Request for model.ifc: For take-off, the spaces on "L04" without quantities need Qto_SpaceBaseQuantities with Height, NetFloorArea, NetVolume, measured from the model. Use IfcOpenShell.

First a look at what the model holds.

```python
import ifcopenshell
import ifcopenshell.util.element
import ifcopenshell.util.unit

model = ifcopenshell.open("model.ifc")
print(model.schema)
for unit_type in ("LENGTHUNIT", "AREAUNIT", "VOLUMEUNIT"):
    print(unit_type, ifcopenshell.util.unit.calculate_unit_scale(model, unit_type))
storey = next(s for s in model.by_type("IfcBuildingStorey") if s.Name == "L04")
spaces = [e for e in ifcopenshell.util.element.get_decomposition(storey) if e.is_a("IfcSpace")]
for e in sorted(spaces, key=lambda e: e.id()):
    print(e.id(), e.is_a(), e.Name, list(ifcopenshell.util.element.get_psets(e, qtos_only=True)), sep=" | ")
```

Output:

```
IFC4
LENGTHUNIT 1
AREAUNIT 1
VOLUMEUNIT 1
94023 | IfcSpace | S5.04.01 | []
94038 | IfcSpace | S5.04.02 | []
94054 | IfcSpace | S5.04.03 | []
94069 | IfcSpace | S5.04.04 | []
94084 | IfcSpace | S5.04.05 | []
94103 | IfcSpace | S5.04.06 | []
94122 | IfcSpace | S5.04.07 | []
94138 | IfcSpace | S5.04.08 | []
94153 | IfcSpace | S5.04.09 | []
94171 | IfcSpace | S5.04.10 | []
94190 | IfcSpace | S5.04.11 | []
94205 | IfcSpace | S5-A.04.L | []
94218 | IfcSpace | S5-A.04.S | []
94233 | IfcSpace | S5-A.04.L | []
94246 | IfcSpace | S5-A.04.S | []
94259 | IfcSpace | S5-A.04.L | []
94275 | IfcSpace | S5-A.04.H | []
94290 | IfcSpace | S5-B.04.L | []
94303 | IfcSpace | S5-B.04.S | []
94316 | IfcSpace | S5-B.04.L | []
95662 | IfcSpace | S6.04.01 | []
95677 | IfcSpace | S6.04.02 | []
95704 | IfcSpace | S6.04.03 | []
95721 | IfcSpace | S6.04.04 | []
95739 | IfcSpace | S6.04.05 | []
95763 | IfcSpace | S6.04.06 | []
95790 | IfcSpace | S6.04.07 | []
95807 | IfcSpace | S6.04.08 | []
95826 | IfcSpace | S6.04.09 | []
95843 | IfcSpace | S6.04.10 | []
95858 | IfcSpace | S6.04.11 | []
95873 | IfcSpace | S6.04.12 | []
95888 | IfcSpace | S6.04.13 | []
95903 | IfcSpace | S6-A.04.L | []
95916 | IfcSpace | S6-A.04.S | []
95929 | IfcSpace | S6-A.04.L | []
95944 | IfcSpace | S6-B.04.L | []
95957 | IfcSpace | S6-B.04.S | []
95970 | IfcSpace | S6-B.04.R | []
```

```python
import ifcopenshell
import ifcopenshell.api.pset
import ifcopenshell.geom
import ifcopenshell.util.element
import ifcopenshell.util.shape
import ifcopenshell.util.unit

model = ifcopenshell.open("model.ifc")
unit_scale = ifcopenshell.util.unit.calculate_unit_scale(model)
area_scale = ifcopenshell.util.unit.calculate_unit_scale(model, "AREAUNIT")
volume_scale = ifcopenshell.util.unit.calculate_unit_scale(model, "VOLUMEUNIT")
settings = ifcopenshell.geom.settings()

storey = next(s for s in model.by_type("IfcBuildingStorey") if s.Name == "L04")
spaces = [e for e in ifcopenshell.util.element.get_decomposition(storey) if e.is_a("IfcSpace")]

for e in sorted(spaces, key=lambda e: e.id()):
    if ifcopenshell.util.element.get_psets(e, qtos_only=True, should_inherit=False):
        continue
    # Geometry comes back in metres, in the element's own axes.
    shape = ifcopenshell.geom.create_shape(settings, e)
    values = {
        "Height": ifcopenshell.util.shape.get_z(shape.geometry) / unit_scale,
        "NetFloorArea": ifcopenshell.util.shape.get_footprint_area(shape.geometry) / area_scale,
        "NetVolume": ifcopenshell.util.shape.get_volume(shape.geometry) / volume_scale,
    }
    qto = ifcopenshell.api.pset.add_qto(model, product=e, name="Qto_SpaceBaseQuantities")
    ifcopenshell.api.pset.edit_qto(model, qto=qto, properties=values)
    print(e.id(), {k: round(v, 3) for k, v in values.items()})

model.write("model-out.ifc")
```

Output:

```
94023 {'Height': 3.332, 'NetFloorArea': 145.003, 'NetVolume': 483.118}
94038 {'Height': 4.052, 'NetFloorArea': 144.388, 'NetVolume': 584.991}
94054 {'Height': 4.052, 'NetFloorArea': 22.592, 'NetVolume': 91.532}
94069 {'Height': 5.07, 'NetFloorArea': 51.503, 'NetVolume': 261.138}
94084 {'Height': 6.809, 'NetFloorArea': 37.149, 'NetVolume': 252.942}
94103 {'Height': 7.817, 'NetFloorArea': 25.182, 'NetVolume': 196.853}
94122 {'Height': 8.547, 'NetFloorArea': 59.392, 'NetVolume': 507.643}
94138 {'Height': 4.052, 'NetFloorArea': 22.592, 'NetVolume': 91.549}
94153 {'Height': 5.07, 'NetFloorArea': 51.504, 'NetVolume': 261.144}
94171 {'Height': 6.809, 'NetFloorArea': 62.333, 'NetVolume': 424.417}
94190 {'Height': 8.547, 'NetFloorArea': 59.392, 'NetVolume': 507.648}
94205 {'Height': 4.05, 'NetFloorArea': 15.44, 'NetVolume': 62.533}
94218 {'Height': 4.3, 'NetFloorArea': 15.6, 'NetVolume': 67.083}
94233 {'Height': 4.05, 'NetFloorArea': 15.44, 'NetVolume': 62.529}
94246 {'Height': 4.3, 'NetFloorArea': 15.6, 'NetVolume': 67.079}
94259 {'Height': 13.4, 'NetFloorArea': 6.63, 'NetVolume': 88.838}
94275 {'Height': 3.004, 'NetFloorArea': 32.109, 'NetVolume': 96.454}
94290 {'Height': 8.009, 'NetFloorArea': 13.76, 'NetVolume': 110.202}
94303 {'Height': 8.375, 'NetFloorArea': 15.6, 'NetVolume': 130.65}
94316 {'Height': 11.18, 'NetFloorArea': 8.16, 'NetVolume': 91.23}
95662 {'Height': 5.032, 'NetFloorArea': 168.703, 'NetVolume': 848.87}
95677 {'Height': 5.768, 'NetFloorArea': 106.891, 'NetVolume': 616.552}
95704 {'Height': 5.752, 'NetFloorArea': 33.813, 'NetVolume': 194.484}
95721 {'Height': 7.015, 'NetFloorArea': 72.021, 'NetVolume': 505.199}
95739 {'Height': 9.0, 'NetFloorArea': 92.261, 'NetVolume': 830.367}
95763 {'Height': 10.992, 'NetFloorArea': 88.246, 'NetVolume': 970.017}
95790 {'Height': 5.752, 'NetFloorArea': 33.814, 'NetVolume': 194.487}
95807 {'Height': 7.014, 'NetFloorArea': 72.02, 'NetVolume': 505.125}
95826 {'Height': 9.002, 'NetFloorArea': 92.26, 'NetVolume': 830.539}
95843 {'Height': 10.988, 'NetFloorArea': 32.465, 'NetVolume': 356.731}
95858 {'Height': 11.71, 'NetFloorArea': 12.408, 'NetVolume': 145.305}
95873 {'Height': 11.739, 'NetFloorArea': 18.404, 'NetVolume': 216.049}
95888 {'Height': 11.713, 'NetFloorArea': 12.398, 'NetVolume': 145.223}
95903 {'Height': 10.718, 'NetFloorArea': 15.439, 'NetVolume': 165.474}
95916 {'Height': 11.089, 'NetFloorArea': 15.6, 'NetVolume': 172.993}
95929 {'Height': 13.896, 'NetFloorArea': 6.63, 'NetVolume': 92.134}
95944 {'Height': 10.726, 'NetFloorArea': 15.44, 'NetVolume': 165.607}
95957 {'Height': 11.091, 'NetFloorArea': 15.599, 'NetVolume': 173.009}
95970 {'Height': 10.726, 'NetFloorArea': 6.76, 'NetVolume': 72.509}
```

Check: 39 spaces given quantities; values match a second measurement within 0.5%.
